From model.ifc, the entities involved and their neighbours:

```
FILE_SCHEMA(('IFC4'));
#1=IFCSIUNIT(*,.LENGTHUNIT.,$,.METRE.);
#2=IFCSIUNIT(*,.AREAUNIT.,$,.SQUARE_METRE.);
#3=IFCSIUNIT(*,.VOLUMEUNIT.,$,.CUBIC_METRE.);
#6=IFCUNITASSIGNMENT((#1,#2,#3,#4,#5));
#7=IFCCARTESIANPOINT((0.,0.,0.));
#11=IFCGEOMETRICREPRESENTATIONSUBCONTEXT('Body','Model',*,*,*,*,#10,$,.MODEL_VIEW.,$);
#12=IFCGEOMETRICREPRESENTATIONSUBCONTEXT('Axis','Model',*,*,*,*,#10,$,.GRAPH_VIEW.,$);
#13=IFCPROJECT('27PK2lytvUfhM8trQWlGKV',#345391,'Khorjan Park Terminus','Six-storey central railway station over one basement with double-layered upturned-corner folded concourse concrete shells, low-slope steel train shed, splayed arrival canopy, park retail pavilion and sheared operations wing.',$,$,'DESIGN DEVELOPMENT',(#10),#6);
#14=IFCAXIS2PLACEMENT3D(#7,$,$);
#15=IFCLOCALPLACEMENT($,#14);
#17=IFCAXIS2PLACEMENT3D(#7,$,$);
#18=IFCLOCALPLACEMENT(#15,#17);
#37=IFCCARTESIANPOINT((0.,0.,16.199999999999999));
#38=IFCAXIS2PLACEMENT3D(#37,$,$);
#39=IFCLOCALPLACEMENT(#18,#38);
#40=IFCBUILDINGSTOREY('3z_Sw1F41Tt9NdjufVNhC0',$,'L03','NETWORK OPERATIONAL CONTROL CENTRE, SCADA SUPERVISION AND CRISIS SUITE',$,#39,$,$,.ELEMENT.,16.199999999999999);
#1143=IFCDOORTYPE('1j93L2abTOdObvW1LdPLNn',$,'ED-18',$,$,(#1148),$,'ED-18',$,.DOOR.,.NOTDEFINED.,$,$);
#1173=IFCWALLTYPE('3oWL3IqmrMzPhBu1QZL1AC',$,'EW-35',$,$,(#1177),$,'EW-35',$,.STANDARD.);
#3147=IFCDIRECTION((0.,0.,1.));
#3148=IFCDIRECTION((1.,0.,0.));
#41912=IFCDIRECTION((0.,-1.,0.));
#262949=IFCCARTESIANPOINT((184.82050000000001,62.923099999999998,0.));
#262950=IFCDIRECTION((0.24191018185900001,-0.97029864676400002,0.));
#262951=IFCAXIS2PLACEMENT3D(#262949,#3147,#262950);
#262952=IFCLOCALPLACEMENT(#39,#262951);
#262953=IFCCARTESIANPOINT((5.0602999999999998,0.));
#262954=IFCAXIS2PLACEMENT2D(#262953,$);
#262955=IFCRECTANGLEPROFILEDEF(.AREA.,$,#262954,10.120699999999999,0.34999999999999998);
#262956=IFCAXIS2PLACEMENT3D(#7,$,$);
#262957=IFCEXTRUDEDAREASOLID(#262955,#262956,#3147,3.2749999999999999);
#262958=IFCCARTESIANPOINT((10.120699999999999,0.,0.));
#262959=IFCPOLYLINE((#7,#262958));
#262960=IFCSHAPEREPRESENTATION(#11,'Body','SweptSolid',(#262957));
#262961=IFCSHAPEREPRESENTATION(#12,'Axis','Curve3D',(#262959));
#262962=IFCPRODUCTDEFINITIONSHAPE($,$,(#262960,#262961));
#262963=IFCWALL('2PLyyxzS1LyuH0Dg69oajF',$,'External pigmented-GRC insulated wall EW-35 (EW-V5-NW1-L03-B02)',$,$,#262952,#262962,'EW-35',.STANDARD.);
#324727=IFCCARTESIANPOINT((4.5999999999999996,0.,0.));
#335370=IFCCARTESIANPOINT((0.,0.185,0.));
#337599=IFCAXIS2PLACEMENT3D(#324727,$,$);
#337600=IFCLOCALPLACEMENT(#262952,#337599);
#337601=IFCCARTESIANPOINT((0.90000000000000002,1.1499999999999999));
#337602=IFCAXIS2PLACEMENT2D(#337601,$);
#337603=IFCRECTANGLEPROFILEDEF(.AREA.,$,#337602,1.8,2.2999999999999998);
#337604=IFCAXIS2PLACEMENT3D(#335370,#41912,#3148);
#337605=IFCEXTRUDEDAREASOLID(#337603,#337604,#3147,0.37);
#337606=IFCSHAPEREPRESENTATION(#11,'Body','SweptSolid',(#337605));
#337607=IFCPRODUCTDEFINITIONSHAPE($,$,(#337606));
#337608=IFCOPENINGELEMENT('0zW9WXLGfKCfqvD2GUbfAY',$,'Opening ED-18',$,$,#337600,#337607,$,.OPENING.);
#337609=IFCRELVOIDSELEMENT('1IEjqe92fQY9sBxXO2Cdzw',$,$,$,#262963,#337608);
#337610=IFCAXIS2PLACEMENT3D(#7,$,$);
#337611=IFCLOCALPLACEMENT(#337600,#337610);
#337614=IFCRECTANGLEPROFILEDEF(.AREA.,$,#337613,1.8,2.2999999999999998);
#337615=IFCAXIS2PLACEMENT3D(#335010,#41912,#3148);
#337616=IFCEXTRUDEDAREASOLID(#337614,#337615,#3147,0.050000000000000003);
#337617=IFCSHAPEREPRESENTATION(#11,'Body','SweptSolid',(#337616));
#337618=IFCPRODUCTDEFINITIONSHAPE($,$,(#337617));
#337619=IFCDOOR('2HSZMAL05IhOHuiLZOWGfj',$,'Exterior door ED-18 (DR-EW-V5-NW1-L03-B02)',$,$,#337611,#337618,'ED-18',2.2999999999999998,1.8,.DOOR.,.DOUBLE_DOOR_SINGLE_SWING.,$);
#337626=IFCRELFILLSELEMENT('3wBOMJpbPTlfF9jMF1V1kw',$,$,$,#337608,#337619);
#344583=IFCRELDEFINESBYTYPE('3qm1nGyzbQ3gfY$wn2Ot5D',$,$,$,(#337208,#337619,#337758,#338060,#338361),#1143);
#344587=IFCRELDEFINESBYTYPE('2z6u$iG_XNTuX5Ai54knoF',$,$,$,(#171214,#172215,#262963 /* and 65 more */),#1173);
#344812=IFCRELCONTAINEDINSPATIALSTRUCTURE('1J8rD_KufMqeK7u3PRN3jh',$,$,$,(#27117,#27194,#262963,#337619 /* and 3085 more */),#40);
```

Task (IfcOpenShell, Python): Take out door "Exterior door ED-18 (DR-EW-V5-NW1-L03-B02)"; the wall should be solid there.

```python
import ifcopenshell
import ifcopenshell.api.feature
import ifcopenshell.api.root
import ifcopenshell.geom
import ifcopenshell.util.shape

model = ifcopenshell.open("model.ifc")
settings = ifcopenshell.geom.settings()


def volume(element):
    """Net volume in cubic metres, openings subtracted."""
    shape = ifcopenshell.geom.create_shape(settings, element)
    return ifcopenshell.util.shape.get_volume(shape.geometry)


door = model.by_guid("2HSZMAL05IhOHuiLZOWGfj")
opening = door.FillsVoids[0].RelatingOpeningElement
wall = opening.VoidsElements[0].RelatingBuildingElement
before = volume(wall)

ifcopenshell.api.root.remove_product(model, product=door)
ifcopenshell.api.feature.remove_feature(model, feature=opening)

after = volume(wall)

print(f"wall volume {before:.3f} -> {after:.3f} m3")

model.write("model_rev.ifc")
```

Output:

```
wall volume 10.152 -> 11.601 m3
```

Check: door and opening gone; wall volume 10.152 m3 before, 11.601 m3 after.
